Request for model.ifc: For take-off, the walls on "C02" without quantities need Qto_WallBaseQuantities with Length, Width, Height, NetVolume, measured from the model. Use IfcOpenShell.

First a look at what the model holds.

```python
import ifcopenshell
import ifcopenshell.util.element
import ifcopenshell.util.unit

model = ifcopenshell.open("model.ifc")
print(model.schema)
for unit_type in ("LENGTHUNIT", "AREAUNIT", "VOLUMEUNIT"):
    print(unit_type, ifcopenshell.util.unit.calculate_unit_scale(model, unit_type))
storey = next(s for s in model.by_type("IfcBuildingStorey") if s.Name == "C02")
walls = [e for e in ifcopenshell.util.element.get_decomposition(storey) if e.is_a("IfcWall")]
for e in sorted(walls, key=lambda e: e.id()):
    print(e.id(), e.is_a(), e.Name, list(ifcopenshell.util.element.get_psets(e, qtos_only=True)), sep=" | ")
```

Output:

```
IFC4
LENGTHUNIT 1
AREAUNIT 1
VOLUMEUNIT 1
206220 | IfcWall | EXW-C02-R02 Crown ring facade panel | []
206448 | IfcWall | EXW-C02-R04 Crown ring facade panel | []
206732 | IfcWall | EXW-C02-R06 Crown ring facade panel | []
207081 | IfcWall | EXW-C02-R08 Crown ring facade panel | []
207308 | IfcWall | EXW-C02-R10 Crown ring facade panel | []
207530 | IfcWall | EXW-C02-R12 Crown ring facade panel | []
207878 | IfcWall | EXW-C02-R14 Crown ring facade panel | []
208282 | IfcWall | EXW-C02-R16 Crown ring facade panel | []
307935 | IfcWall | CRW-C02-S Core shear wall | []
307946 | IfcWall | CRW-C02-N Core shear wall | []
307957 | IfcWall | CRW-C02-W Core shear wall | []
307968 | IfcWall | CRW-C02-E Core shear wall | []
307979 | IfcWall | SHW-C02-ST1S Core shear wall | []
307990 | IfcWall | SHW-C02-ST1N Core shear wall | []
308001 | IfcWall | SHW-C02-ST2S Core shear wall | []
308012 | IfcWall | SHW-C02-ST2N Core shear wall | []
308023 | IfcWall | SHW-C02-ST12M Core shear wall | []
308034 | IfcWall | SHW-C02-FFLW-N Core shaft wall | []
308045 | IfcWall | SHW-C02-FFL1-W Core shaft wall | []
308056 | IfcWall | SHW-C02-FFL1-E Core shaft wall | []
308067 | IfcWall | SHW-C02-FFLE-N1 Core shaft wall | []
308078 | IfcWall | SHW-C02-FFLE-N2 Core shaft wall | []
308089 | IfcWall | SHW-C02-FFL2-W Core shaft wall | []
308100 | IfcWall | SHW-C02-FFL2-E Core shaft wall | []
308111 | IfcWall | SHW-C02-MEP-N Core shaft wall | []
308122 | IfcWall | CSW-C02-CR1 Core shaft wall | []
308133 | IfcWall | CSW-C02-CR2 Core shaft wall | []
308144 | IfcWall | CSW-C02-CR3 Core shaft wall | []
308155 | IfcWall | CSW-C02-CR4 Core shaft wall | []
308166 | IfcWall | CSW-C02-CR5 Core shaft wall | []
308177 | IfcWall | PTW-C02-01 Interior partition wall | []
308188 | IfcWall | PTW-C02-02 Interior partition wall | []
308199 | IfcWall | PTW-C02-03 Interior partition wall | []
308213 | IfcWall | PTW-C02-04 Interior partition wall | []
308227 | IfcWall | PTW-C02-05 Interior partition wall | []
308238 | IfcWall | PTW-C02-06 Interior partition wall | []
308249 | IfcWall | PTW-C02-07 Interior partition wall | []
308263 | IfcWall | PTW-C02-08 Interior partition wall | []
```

```python
import ifcopenshell
import ifcopenshell.api.pset
import ifcopenshell.geom
import ifcopenshell.util.element
import ifcopenshell.util.shape
import ifcopenshell.util.unit

model = ifcopenshell.open("model.ifc")
unit_scale = ifcopenshell.util.unit.calculate_unit_scale(model)
volume_scale = ifcopenshell.util.unit.calculate_unit_scale(model, "VOLUMEUNIT")
settings = ifcopenshell.geom.settings()

storey = next(s for s in model.by_type("IfcBuildingStorey") if s.Name == "C02")
walls = [e for e in ifcopenshell.util.element.get_decomposition(storey) if e.is_a("IfcWall")]

for e in sorted(walls, key=lambda e: e.id()):
    if ifcopenshell.util.element.get_psets(e, qtos_only=True, should_inherit=False):
        continue
    # Geometry comes back in metres, in the element's own axes.
    shape = ifcopenshell.geom.create_shape(settings, e)
    values = {
        "Length": ifcopenshell.util.shape.get_x(shape.geometry) / unit_scale,
        "Width": ifcopenshell.util.shape.get_y(shape.geometry) / unit_scale,
        "Height": ifcopenshell.util.shape.get_z(shape.geometry) / unit_scale,
        "NetVolume": ifcopenshell.util.shape.get_volume(shape.geometry) / volume_scale,
    }
    qto = ifcopenshell.api.pset.add_qto(model, product=e, name="Qto_WallBaseQuantities")
    ifcopenshell.api.pset.edit_qto(model, qto=qto, properties=values)
    print(e.id(), {k: round(v, 3) for k, v in values.items()})

model.write("model_rev.ifc")
```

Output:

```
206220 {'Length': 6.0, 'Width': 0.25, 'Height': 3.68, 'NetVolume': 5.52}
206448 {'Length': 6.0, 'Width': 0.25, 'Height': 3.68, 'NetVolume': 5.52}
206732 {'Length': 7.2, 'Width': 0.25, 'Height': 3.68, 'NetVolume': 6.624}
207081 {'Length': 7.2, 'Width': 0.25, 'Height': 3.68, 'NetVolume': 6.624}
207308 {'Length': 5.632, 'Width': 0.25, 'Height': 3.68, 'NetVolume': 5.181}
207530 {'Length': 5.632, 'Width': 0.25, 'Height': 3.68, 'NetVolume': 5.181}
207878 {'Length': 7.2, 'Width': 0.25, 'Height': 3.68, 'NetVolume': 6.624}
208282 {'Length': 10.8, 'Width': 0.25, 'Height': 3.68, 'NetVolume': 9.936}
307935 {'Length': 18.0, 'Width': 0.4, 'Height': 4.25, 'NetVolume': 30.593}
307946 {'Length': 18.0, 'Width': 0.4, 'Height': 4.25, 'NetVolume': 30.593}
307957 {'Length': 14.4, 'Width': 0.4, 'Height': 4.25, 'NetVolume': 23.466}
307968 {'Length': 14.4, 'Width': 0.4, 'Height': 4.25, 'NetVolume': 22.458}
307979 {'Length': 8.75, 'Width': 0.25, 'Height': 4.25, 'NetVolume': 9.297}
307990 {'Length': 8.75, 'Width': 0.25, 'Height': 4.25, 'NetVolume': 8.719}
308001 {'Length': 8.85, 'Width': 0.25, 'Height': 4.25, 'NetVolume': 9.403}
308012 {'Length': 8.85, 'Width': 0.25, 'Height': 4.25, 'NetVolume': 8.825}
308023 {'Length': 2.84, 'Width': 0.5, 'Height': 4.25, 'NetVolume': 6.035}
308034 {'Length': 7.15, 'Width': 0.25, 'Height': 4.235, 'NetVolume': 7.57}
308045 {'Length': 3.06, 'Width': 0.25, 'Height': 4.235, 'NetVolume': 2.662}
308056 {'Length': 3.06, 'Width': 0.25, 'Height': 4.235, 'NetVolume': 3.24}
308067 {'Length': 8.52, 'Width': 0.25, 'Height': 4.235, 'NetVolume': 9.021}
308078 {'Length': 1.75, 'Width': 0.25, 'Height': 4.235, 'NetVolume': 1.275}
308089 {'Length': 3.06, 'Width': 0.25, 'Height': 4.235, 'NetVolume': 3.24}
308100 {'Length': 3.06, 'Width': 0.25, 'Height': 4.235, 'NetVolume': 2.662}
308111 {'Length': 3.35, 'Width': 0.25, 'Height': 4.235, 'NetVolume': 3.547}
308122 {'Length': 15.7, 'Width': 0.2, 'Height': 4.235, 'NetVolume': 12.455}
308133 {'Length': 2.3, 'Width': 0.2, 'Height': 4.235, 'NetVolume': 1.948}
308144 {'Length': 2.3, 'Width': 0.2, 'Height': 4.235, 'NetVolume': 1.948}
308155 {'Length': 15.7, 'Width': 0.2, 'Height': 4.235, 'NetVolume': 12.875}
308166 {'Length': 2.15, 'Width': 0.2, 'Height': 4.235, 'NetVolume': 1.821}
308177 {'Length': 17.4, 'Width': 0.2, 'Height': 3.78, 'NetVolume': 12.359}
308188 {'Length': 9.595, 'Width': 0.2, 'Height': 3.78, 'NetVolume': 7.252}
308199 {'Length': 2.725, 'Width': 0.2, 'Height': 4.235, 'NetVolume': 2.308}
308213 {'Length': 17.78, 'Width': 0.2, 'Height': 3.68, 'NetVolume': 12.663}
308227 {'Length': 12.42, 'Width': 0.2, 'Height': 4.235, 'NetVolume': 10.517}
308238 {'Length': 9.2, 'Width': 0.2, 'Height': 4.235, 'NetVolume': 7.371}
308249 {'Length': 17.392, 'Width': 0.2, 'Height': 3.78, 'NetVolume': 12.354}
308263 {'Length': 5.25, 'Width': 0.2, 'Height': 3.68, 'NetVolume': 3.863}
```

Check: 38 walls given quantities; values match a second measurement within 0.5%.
